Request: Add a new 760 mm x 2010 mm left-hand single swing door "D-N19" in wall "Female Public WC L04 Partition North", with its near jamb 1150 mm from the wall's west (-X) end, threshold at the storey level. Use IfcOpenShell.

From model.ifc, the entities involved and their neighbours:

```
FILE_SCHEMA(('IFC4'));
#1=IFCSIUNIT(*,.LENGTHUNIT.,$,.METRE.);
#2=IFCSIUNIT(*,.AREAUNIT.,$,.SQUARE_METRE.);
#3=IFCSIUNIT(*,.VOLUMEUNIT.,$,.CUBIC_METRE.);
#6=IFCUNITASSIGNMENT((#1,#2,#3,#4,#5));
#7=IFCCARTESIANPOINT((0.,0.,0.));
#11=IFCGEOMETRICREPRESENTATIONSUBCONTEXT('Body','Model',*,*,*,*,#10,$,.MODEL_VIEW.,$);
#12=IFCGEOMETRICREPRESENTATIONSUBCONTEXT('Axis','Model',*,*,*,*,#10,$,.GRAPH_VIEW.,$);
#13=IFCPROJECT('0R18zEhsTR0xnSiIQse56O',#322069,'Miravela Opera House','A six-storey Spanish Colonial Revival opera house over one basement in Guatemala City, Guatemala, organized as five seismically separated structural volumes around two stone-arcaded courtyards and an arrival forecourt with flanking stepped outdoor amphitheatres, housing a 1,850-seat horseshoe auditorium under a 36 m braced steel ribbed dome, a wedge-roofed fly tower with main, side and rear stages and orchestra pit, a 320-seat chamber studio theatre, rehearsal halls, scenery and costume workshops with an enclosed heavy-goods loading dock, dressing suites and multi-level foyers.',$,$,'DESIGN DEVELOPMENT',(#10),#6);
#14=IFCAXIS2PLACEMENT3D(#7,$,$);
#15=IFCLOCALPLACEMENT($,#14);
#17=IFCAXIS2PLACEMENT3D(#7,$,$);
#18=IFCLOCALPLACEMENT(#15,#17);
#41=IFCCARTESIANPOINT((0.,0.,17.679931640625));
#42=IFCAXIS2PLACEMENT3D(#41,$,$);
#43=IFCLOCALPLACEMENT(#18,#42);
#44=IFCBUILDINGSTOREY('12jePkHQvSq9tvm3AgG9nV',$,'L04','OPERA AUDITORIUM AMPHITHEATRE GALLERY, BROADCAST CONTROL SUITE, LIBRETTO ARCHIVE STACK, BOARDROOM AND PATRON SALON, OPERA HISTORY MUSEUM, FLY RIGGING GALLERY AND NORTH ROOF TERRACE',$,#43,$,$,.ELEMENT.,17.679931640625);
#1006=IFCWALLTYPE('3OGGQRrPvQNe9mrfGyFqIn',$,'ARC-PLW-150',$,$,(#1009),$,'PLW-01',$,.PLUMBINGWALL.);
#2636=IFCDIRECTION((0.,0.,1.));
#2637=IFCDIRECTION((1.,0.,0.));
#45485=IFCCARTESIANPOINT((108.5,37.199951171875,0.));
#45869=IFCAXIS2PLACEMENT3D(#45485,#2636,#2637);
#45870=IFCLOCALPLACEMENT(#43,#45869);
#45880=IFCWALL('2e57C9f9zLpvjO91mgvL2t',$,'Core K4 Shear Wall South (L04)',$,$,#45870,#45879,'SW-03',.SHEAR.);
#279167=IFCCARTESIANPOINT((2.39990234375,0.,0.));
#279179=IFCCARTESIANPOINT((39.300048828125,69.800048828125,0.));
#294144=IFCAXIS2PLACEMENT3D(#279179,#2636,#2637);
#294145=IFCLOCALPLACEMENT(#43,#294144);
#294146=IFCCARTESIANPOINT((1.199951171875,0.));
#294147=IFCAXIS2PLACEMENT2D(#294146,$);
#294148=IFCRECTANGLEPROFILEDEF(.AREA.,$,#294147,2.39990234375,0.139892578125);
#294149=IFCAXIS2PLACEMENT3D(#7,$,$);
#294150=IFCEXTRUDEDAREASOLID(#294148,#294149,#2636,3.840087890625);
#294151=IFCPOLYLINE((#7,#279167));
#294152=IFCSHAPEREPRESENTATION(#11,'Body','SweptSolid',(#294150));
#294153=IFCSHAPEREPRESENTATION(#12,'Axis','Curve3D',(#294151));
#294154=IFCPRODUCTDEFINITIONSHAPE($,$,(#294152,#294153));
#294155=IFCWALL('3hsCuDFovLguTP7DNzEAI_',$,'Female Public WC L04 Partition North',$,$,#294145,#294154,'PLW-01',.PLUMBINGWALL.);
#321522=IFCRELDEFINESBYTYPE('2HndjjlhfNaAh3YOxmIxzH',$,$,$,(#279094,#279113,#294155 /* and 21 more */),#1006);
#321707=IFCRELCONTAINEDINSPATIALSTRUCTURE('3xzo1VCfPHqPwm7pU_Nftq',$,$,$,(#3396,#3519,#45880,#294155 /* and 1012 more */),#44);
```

```python
import numpy as np
import ifcopenshell
import ifcopenshell.api.feature
import ifcopenshell.api.geometry
import ifcopenshell.api.root
import ifcopenshell.api.spatial
import ifcopenshell.geom
import ifcopenshell.util.element
import ifcopenshell.util.placement
import ifcopenshell.util.representation
import ifcopenshell.util.shape
import ifcopenshell.util.unit

model = ifcopenshell.open("model.ifc")
unit_scale = ifcopenshell.util.unit.calculate_unit_scale(model)
settings = ifcopenshell.geom.settings()


def volume(element):
    """Net volume in cubic metres, openings subtracted."""
    shape = ifcopenshell.geom.create_shape(settings, element)
    return ifcopenshell.util.shape.get_volume(shape.geometry)


wall = model.by_guid("3hsCuDFovLguTP7DNzEAI_")
storey = ifcopenshell.util.element.get_container(wall, ifc_class="IfcBuildingStorey")
context = ifcopenshell.util.representation.get_context(model, "Model", "Body", "MODEL_VIEW")
before = volume(wall)

width, height, from_end, sill = 0.76, 2.01, 1.15, 0.0  # metres

# The wall runs along its own X axis, and the end named is its -X end.
wall_shape = ifcopenshell.geom.create_shape(settings, wall)
x, y, z = ifcopenshell.util.shape.get_vertices(wall_shape.geometry).T
start = x.min() + from_end
face, thickness = float(y.min()), float(y.max() - y.min())
wall_matrix = ifcopenshell.util.placement.get_local_placement(wall.ObjectPlacement)
level = ifcopenshell.util.placement.get_local_placement(storey.ObjectPlacement)[2, 3]


def in_wall(x, y):
    """Placement at x, y metres in the wall's axes, at sill height."""
    matrix = wall_matrix.copy()
    matrix[:, 3] = wall_matrix @ np.array([x / unit_scale, y / unit_scale, 0.0, 1.0])
    matrix[2, 3] = level + sill / unit_scale
    return matrix


# Opening: a box that overshoots both wall faces by 50 mm.
opening = ifcopenshell.api.root.create_entity(model, ifc_class="IfcOpeningElement", predefined_type="OPENING")
box = ifcopenshell.api.geometry.add_wall_representation(
    model, context=context, length=width, height=height, thickness=thickness + 0.1
)
ifcopenshell.api.geometry.assign_representation(model, product=opening, representation=box)
ifcopenshell.api.geometry.edit_object_placement(model, product=opening, matrix=in_wall(start, face - 0.05), is_si=False)
ifcopenshell.api.feature.add_feature(model, feature=opening, element=wall)

door = ifcopenshell.api.root.create_entity(model, ifc_class="IfcDoor", name="D-N19", predefined_type="DOOR")
door.OverallWidth, door.OverallHeight = width / unit_scale, height / unit_scale
door.OperationType = "SINGLE_SWING_LEFT"
body = ifcopenshell.api.geometry.add_door_representation(
    model,
    context=context,
    overall_width=door.OverallWidth,
    overall_height=door.OverallHeight,
    operation_type="SINGLE_SWING_LEFT",
    lining_properties={"LiningDepth": thickness / unit_scale, "ThresholdDepth": thickness / unit_scale},
)
ifcopenshell.api.geometry.assign_representation(model, product=door, representation=body)
ifcopenshell.api.spatial.assign_container(model, products=[door], relating_structure=storey)
ifcopenshell.api.feature.add_filling(model, opening=opening, element=door)

# The lining spans the wall, so the door starts at the wall face.
ifcopenshell.api.geometry.edit_object_placement(model, product=door, matrix=in_wall(start, face), is_si=False)

after = volume(wall)

print(f"wall volume {before:.3f} -> {after:.3f} m3")

model.write("model_edited.ifc")
```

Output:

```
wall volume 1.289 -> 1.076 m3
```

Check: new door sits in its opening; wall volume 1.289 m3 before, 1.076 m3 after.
